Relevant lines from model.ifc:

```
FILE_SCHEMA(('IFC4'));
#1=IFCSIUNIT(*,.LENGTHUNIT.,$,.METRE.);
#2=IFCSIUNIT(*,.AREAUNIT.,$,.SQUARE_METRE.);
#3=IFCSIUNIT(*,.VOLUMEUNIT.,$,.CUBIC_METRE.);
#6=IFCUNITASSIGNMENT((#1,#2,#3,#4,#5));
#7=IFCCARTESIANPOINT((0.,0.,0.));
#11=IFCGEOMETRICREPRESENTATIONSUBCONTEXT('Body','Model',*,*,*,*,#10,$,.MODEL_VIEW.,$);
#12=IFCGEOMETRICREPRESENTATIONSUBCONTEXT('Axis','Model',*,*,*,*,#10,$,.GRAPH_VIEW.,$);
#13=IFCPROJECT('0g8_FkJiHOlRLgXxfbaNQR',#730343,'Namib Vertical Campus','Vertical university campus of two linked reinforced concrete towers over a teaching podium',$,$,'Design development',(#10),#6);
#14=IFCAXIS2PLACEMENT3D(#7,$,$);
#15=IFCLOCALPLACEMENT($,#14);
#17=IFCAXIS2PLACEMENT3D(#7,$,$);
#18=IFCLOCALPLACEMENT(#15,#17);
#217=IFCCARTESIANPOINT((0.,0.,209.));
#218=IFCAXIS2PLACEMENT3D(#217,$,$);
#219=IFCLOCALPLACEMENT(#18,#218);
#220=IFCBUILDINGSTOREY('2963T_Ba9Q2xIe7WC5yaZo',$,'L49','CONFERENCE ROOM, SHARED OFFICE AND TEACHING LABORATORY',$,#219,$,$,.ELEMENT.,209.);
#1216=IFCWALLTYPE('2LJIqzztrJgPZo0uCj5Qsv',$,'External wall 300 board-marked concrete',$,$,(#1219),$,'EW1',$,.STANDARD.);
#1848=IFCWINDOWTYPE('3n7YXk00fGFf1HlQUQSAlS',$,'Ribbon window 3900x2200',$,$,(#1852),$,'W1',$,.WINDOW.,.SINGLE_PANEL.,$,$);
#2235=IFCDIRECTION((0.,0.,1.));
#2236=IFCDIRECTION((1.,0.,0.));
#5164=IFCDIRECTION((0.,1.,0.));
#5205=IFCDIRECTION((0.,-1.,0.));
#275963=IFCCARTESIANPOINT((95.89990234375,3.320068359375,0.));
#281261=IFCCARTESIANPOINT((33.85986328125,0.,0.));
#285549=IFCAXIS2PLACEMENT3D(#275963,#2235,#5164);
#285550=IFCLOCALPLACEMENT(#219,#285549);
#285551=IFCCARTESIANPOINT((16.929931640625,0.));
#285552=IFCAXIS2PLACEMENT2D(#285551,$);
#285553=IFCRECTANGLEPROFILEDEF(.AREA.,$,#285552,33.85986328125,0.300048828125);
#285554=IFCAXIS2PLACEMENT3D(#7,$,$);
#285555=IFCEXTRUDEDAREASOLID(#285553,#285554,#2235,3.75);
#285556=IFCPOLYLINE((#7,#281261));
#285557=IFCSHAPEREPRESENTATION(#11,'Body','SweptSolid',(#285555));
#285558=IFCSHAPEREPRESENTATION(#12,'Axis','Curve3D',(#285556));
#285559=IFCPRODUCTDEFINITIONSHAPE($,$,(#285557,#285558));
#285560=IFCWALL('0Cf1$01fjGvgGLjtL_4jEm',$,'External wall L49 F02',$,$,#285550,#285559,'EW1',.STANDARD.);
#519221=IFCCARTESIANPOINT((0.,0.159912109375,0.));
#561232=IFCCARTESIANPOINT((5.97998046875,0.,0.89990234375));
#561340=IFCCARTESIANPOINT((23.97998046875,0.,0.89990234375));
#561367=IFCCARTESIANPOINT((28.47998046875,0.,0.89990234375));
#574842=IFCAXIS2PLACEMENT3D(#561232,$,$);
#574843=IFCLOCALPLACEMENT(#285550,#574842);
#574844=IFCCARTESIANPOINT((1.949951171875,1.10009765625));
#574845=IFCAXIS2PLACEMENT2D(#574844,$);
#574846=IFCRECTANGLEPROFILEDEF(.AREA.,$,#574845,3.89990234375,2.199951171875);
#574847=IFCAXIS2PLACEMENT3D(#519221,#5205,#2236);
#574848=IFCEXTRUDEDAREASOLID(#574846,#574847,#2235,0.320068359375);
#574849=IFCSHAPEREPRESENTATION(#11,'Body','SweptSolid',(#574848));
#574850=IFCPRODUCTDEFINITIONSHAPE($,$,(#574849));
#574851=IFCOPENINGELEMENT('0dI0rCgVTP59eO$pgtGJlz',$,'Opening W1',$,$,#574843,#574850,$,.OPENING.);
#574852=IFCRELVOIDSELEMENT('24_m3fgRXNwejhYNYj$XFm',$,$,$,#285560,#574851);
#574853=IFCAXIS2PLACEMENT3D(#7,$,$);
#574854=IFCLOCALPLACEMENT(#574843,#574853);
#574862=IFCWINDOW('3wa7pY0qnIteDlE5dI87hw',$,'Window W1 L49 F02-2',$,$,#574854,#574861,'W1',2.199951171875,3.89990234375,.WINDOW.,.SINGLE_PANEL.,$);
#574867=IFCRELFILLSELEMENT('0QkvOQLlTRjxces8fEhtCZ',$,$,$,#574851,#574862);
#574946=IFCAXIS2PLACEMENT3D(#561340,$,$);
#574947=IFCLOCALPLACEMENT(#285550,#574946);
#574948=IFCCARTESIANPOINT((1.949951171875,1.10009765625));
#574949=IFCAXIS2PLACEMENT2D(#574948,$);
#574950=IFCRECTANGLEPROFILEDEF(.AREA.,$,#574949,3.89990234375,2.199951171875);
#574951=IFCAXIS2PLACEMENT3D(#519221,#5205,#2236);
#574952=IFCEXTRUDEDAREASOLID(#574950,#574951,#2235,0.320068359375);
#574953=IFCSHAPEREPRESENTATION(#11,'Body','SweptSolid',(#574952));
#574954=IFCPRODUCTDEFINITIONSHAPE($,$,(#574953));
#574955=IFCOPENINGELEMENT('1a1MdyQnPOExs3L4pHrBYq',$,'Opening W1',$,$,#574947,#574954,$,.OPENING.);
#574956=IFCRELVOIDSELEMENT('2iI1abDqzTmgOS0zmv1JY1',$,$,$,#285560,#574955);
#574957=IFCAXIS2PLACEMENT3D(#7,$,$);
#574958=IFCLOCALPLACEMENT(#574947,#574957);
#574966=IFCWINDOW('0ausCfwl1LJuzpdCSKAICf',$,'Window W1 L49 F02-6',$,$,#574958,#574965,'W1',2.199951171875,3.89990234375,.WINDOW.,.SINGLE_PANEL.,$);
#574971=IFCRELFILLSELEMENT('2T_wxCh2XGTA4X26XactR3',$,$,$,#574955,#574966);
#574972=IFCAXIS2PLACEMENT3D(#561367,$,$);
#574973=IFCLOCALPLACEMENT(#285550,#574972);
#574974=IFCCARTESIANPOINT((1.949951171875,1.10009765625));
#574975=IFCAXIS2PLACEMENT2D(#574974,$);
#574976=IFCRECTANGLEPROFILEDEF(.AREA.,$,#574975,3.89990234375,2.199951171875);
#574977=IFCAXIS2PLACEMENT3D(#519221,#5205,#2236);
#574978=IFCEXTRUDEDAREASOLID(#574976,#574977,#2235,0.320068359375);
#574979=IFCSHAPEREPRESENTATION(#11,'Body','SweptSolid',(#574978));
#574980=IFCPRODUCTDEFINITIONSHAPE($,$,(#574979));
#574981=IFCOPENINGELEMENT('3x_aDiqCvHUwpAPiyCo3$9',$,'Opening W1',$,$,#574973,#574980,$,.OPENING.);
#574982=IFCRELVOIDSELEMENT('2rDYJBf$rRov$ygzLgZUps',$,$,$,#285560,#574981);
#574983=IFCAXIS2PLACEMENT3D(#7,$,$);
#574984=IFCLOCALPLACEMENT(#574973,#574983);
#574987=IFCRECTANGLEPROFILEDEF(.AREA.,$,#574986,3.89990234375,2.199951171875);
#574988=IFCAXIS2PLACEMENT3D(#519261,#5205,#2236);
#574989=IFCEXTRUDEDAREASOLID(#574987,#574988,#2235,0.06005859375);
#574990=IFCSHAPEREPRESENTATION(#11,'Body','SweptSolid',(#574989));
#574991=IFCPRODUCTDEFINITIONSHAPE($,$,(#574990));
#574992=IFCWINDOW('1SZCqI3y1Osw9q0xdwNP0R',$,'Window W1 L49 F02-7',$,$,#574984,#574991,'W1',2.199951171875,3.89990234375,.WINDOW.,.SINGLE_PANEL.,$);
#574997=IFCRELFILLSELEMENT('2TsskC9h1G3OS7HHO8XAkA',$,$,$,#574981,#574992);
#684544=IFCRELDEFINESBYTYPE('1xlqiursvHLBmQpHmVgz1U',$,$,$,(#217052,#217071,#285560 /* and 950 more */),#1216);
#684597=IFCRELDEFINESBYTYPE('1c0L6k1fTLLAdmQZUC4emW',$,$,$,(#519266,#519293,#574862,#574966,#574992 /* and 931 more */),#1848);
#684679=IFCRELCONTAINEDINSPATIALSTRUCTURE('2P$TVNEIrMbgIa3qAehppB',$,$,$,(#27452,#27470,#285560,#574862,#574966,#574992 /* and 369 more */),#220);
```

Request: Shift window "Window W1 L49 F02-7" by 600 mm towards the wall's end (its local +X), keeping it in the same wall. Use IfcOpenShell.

```python
import ifcopenshell
import ifcopenshell.api.geometry
import ifcopenshell.util.placement
import ifcopenshell.util.unit

model = ifcopenshell.open("model.ifc")
unit_scale = ifcopenshell.util.unit.calculate_unit_scale(model)

window = model.by_id(574992)
opening = window.FillsVoids[0].RelatingOpeningElement
wall = opening.VoidsElements[0].RelatingBuildingElement

wall_matrix = ifcopenshell.util.placement.get_local_placement(wall.ObjectPlacement)
shift = wall_matrix[:3, 0] * 0.6 / unit_scale
before = ifcopenshell.util.placement.get_local_placement(window.ObjectPlacement)[:3, 3].copy()

# The window is placed relative to its opening, so it follows when the opening moves.
matrix = ifcopenshell.util.placement.get_local_placement(opening.ObjectPlacement)
matrix[:3, 3] += shift
ifcopenshell.api.geometry.edit_object_placement(
    model, product=opening, matrix=matrix, is_si=False, should_transform_children=True
)

after = ifcopenshell.util.placement.get_local_placement(window.ObjectPlacement)[:3, 3]
print("window moved by", (after - before).round(3) + 0.0)

model.write("model_edited.ifc")
```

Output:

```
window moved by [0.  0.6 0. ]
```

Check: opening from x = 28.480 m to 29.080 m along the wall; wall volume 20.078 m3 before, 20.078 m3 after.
